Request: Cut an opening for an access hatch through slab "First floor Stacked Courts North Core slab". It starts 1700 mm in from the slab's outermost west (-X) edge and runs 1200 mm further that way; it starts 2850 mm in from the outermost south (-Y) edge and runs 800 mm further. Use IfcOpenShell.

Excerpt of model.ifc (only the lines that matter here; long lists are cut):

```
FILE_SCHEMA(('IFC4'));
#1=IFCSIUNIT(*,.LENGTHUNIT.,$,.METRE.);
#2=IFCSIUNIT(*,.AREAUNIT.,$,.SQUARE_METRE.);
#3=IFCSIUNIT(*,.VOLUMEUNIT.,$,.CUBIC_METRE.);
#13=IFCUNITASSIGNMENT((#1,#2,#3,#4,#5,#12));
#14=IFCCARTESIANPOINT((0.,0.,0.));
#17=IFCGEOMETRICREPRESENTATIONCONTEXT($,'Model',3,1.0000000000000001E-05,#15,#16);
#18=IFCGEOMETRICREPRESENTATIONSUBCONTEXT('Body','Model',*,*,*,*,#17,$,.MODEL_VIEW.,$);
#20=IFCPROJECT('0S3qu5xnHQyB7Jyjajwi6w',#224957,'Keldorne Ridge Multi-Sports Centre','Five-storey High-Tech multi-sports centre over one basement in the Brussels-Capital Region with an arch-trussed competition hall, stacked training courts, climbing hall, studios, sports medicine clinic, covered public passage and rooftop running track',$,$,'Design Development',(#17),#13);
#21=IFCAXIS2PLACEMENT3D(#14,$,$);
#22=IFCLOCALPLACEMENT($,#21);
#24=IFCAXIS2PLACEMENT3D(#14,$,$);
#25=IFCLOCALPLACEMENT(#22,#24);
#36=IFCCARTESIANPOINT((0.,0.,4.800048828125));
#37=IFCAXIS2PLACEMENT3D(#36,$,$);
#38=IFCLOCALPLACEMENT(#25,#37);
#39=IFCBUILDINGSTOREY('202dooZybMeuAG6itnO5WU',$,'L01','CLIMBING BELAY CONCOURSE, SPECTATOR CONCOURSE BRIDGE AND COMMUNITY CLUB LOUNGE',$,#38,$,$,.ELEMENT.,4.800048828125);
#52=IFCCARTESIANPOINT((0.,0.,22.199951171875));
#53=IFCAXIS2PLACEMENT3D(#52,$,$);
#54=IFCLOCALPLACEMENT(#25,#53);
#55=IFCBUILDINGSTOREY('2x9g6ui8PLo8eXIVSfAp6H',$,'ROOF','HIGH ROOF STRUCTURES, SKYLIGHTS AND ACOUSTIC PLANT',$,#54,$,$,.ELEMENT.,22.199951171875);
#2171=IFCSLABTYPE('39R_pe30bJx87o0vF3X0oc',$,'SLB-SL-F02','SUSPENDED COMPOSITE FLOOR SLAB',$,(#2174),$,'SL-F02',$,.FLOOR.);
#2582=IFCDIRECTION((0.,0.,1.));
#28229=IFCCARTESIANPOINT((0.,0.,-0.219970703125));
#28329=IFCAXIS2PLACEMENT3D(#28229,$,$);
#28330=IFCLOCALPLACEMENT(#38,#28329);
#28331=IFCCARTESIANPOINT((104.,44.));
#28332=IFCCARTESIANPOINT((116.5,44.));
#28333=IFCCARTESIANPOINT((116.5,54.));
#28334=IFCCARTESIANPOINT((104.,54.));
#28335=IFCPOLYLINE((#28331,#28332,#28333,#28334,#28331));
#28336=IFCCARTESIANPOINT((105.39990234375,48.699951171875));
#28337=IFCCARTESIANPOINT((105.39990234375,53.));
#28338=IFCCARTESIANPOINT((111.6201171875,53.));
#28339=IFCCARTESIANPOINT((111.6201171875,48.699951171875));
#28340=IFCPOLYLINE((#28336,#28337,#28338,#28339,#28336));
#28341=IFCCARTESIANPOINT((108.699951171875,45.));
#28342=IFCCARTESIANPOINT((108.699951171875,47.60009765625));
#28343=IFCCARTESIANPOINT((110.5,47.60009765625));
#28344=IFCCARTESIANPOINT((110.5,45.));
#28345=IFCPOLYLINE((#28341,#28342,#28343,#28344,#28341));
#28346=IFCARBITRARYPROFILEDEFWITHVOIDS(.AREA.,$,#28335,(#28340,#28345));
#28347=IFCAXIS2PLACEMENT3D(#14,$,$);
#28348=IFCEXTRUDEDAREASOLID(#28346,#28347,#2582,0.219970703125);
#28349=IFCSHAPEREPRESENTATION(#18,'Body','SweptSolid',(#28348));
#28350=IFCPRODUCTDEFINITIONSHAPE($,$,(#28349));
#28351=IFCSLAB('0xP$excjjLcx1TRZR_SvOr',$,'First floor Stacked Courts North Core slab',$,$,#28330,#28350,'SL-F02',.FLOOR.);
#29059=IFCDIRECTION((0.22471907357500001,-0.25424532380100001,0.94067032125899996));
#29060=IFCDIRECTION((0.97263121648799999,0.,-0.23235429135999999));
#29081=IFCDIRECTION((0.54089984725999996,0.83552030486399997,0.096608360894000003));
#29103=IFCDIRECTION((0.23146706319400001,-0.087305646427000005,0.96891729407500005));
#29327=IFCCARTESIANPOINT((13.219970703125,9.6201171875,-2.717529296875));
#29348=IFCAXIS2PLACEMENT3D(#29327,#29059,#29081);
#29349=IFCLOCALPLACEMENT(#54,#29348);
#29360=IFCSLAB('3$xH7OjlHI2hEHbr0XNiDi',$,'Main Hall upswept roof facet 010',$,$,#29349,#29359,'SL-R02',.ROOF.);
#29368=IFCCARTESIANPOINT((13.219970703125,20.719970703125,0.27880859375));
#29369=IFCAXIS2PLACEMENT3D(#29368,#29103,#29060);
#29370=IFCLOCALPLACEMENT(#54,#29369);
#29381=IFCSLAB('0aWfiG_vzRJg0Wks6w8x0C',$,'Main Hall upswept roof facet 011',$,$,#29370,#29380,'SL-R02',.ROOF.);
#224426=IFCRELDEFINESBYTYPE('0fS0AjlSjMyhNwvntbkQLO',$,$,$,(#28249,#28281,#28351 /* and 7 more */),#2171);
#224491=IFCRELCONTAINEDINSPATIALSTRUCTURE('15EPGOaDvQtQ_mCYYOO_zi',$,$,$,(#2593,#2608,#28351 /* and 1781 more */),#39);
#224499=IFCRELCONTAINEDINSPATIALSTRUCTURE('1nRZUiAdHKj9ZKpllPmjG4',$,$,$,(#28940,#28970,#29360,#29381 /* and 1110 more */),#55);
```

```python
import numpy as np
import ifcopenshell
import ifcopenshell.api.feature
import ifcopenshell.api.geometry
import ifcopenshell.api.root
import ifcopenshell.geom
import ifcopenshell.util.placement
import ifcopenshell.util.representation
import ifcopenshell.util.shape
import ifcopenshell.util.unit

model = ifcopenshell.open("model.ifc")
unit_scale = ifcopenshell.util.unit.calculate_unit_scale(model)
settings = ifcopenshell.geom.settings()


def volume(element):
    """Net volume in cubic metres, openings subtracted."""
    shape = ifcopenshell.geom.create_shape(settings, element)
    return ifcopenshell.util.shape.get_volume(shape.geometry)


slab = model.by_guid("0xP$excjjLcx1TRZR_SvOr")
before = volume(slab)

# Extent in the slab's own axes, in metres. The edges named are its -X and -Y sides.
slab_shape = ifcopenshell.geom.create_shape(settings, slab)
vertices = ifcopenshell.util.shape.get_vertices(slab_shape.geometry)
x_min, y_min, bottom = vertices.min(axis=0)
top = vertices[:, 2].max()

opening = ifcopenshell.api.root.create_entity(model, ifc_class="IfcOpeningElement", name="Access hatch opening", predefined_type="OPENING")
context = ifcopenshell.util.representation.get_context(model, "Model", "Body", "MODEL_VIEW")
width, depth = 1.2, 0.8
outline = [(0.0, 0.0), (width, 0.0), (width, depth), (0.0, depth), (0.0, 0.0)]
# Overshoot both faces by 50 mm so the cut is clean.
shape = ifcopenshell.api.geometry.add_slab_representation(
    model, context=context, depth=top - bottom + 0.1, polyline=outline
)
ifcopenshell.api.geometry.assign_representation(model, product=opening, representation=shape)

matrix = ifcopenshell.util.placement.get_local_placement(slab.ObjectPlacement)
matrix[:, 3] = matrix @ np.append(np.array([x_min + 1.7, y_min + 2.85, bottom - 0.05]) / unit_scale, 1.0)
ifcopenshell.api.geometry.edit_object_placement(model, product=opening, matrix=matrix, is_si=False)
ifcopenshell.api.feature.add_feature(model, feature=opening, element=slab)

after = volume(slab)

print(f"slab volume {before:.3f} -> {after:.3f} m3")

model.write("model_edited.ifc")
```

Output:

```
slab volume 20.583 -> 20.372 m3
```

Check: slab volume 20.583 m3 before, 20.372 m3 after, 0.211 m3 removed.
